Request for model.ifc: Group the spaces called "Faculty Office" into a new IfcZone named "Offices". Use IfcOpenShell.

First a look at what the model holds.

```python
import ifcopenshell

model = ifcopenshell.open("model.ifc")
print(model.schema)
seen = {}
for space in model.by_type("IfcSpace"):
    seen[space.LongName] = seen.get(space.LongName, 0) + 1
for name, count in sorted(seen.items(), key=str):
    print(count, "x", name)
print("zones:", [z.Name for z in model.by_type("IfcZone")][:20])
```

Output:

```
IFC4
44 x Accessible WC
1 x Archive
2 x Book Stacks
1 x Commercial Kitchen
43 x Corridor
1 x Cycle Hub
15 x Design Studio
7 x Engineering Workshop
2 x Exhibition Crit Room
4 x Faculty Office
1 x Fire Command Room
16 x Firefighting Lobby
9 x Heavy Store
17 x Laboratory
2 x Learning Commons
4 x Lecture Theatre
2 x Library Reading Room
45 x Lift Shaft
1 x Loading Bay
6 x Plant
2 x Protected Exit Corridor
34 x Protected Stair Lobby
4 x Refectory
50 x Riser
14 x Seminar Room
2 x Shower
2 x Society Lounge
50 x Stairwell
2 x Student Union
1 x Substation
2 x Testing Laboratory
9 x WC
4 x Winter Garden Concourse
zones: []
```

```python
import ifcopenshell
import ifcopenshell.api.group
import ifcopenshell.api.root

model = ifcopenshell.open("model.ifc")

names = {"Faculty Office"}
spaces = [s for s in model.by_type("IfcSpace") if s.LongName in names]

zone = ifcopenshell.api.root.create_entity(model, ifc_class="IfcZone", name="Offices")
ifcopenshell.api.group.assign_group(model, products=spaces, group=zone)
print(len(spaces), "spaces in", zone.Name)

model.write("model_edited.ifc")
```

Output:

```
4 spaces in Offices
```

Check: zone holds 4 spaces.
